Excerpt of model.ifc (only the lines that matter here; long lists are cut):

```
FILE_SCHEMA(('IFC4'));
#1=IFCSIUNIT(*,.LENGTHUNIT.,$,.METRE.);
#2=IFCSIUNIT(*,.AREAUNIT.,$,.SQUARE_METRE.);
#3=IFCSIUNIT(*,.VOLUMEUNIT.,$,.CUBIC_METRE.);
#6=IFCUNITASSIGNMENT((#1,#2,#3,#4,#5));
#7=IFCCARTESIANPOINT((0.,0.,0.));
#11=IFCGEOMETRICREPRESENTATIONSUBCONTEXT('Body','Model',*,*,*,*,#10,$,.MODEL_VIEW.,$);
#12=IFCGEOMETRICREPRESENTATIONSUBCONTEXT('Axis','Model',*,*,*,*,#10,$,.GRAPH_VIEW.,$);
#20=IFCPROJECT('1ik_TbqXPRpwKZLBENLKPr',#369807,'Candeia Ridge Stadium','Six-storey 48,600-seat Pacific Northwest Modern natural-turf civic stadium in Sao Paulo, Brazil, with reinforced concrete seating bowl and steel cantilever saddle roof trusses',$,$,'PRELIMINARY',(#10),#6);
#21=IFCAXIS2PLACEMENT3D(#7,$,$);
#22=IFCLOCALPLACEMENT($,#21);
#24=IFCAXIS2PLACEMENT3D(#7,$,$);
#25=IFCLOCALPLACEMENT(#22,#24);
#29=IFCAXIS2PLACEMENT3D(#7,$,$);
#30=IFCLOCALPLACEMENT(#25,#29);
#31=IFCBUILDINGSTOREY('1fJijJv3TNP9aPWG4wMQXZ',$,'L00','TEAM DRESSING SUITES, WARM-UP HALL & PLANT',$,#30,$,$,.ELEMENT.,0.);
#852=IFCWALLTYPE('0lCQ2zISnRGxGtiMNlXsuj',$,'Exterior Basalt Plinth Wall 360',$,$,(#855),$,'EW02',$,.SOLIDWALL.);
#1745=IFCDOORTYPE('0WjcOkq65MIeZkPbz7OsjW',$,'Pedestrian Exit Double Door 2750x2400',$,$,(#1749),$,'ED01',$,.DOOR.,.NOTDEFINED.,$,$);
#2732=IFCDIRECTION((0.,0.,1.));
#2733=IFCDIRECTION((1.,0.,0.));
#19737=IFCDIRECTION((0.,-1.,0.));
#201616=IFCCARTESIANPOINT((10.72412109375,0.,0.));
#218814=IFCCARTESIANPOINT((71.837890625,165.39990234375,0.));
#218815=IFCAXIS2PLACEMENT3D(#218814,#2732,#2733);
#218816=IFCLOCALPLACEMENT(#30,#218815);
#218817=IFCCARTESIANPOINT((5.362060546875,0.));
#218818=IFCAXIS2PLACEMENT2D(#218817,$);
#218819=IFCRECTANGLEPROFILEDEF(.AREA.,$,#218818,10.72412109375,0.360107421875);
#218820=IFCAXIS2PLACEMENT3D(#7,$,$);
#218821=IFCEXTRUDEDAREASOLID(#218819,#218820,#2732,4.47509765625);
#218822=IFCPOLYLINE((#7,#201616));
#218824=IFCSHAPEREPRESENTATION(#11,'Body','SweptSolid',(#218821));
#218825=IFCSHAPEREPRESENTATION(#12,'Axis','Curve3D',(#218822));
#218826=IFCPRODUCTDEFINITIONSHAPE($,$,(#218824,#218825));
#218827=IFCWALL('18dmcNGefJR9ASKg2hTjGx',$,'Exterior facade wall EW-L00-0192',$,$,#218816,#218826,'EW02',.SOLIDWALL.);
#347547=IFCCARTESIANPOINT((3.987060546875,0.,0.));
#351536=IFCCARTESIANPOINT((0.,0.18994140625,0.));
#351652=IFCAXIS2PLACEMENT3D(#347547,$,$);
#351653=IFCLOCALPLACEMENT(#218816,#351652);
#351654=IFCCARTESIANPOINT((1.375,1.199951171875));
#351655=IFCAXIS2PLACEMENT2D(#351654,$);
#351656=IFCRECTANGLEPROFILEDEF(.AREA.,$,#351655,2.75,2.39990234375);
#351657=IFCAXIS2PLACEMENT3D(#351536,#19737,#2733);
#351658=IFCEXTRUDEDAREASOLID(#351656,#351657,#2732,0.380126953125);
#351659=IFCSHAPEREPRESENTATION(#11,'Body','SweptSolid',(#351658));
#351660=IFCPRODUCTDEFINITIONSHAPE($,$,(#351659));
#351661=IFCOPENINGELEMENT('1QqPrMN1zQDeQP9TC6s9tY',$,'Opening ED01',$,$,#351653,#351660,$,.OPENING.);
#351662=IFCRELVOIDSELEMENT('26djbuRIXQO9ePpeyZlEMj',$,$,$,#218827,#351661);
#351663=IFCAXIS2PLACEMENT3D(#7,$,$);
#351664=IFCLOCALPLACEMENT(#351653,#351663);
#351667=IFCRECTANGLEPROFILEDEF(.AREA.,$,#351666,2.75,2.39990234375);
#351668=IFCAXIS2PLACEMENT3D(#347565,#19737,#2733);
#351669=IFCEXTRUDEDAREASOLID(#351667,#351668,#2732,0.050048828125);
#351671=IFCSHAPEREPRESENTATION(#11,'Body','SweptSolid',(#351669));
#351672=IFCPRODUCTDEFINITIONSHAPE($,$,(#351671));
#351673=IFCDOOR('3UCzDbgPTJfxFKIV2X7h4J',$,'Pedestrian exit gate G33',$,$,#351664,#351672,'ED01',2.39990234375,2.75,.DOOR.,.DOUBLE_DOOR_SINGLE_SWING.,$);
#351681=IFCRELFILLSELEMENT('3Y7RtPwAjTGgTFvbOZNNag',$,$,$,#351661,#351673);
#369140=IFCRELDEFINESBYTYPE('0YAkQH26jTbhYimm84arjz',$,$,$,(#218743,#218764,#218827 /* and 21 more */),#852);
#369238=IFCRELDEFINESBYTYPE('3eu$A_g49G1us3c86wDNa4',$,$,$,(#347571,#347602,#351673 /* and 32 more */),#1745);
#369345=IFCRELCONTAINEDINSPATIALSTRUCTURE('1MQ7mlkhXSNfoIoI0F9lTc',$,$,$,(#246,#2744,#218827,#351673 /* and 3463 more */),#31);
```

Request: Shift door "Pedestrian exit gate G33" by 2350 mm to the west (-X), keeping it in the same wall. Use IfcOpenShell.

```python
import ifcopenshell
import ifcopenshell.api.geometry
import ifcopenshell.util.placement
import ifcopenshell.util.unit

model = ifcopenshell.open("model.ifc")
unit_scale = ifcopenshell.util.unit.calculate_unit_scale(model)

door = model.by_guid("3UCzDbgPTJfxFKIV2X7h4J")
opening = door.FillsVoids[0].RelatingOpeningElement
wall = opening.VoidsElements[0].RelatingBuildingElement

wall_matrix = ifcopenshell.util.placement.get_local_placement(wall.ObjectPlacement)
shift = wall_matrix[:3, 0] * -2.35 / unit_scale
before = ifcopenshell.util.placement.get_local_placement(door.ObjectPlacement)[:3, 3].copy()

# The door is placed relative to its opening, so it follows when the opening moves.
matrix = ifcopenshell.util.placement.get_local_placement(opening.ObjectPlacement)
matrix[:3, 3] += shift
ifcopenshell.api.geometry.edit_object_placement(
    model, product=opening, matrix=matrix, is_si=False, should_transform_children=True
)

after = ifcopenshell.util.placement.get_local_placement(door.ObjectPlacement)[:3, 3]
print("door moved by", (after - before).round(3) + 0.0)

model.write("model_v2.ifc")
```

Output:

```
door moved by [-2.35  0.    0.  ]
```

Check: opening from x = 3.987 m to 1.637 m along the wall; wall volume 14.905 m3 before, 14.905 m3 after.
